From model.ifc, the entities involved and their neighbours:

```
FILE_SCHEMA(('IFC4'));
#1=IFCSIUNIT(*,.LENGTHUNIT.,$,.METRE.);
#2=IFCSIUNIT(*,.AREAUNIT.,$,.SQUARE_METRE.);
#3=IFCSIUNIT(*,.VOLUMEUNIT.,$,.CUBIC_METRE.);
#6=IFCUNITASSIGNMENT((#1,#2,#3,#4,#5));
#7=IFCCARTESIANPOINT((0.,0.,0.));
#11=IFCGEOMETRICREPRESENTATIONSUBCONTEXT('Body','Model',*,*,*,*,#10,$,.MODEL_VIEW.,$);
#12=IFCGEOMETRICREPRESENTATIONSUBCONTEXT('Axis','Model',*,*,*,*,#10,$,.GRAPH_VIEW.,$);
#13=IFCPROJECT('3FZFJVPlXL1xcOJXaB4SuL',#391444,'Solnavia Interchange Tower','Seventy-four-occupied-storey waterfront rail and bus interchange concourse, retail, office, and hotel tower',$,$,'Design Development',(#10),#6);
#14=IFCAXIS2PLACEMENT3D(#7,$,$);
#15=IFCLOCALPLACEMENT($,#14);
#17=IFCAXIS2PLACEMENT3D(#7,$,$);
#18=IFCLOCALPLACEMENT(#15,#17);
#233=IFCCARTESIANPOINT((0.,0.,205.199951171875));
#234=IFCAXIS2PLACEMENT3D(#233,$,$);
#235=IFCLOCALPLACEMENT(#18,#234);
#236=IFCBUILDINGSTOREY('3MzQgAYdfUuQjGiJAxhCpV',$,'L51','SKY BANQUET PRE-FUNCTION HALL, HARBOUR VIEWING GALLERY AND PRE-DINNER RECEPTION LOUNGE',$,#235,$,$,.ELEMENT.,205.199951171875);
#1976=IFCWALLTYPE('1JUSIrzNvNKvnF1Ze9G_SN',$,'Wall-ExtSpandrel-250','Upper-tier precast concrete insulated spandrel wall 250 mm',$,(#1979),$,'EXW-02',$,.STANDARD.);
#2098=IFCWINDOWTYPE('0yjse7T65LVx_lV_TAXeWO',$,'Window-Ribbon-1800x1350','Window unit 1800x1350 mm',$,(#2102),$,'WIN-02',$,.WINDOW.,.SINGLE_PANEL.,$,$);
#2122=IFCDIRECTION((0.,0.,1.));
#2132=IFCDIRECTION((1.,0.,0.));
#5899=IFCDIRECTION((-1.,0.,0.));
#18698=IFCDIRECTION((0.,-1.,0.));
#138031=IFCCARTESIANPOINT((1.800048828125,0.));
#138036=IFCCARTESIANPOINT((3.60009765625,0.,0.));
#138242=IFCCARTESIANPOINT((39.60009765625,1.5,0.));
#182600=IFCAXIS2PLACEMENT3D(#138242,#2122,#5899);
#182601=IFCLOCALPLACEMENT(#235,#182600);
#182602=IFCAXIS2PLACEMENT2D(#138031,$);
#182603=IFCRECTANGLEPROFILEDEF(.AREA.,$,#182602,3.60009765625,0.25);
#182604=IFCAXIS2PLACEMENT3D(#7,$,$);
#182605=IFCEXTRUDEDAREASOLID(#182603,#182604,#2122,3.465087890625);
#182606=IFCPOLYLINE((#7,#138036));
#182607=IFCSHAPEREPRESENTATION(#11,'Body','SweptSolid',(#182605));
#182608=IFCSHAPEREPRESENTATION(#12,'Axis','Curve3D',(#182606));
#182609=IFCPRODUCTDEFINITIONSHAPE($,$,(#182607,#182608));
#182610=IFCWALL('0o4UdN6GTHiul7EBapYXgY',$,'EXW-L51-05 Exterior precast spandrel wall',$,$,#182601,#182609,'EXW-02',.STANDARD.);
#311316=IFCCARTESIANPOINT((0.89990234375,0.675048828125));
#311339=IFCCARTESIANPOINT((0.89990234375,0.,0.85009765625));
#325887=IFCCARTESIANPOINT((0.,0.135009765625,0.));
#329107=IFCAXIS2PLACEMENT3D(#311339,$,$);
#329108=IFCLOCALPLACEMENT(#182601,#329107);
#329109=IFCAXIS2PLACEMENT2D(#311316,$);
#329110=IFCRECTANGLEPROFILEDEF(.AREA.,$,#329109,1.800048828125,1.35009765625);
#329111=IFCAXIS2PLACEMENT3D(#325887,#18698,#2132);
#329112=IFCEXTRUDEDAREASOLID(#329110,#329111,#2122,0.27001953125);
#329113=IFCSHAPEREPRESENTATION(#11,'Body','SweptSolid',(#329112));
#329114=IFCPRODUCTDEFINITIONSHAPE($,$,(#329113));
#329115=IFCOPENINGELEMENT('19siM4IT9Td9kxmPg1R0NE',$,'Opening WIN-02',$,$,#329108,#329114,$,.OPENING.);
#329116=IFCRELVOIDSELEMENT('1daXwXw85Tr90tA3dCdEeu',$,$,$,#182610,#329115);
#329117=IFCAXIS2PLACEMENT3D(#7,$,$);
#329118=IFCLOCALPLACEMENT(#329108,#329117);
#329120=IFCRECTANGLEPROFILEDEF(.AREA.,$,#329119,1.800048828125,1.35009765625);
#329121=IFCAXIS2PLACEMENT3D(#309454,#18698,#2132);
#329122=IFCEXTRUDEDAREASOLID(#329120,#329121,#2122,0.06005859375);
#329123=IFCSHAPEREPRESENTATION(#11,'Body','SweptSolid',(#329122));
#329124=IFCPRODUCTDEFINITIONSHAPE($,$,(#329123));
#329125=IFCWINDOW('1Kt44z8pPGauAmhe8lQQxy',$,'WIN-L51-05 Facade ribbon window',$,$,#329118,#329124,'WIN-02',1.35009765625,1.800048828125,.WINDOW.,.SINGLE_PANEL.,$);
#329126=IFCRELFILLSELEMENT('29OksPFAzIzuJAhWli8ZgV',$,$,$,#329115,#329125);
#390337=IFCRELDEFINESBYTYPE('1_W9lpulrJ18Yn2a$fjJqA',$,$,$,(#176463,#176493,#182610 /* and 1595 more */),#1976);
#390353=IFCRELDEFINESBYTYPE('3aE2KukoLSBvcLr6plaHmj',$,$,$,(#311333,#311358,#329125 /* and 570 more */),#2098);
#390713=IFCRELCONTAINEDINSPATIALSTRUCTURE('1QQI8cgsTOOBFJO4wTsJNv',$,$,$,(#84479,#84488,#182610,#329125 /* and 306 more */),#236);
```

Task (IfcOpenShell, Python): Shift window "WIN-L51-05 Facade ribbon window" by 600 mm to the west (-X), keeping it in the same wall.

```python
import ifcopenshell
import ifcopenshell.api.geometry
import ifcopenshell.util.placement

model = ifcopenshell.open("model.ifc")

window = model.by_id(329125)
opening = window.FillsVoids[0].RelatingOpeningElement
wall = opening.VoidsElements[0].RelatingBuildingElement

wall_matrix = ifcopenshell.util.placement.get_local_placement(wall.ObjectPlacement)
shift = wall_matrix[:3, 0] * 0.6
before = ifcopenshell.util.placement.get_local_placement(window.ObjectPlacement)[:3, 3].copy()

# The window is placed relative to its opening, so it follows when the opening moves.
matrix = ifcopenshell.util.placement.get_local_placement(opening.ObjectPlacement)
matrix[:3, 3] += shift
ifcopenshell.api.geometry.edit_object_placement(
    model, product=opening, matrix=matrix, is_si=False, should_transform_children=True
)

after = ifcopenshell.util.placement.get_local_placement(window.ObjectPlacement)[:3, 3]
print("window moved by", (after - before).round(3) + 0.0)

model.write("model_rev.ifc")
```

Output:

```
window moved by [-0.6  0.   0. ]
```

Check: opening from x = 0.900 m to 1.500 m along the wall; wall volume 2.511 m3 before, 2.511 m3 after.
